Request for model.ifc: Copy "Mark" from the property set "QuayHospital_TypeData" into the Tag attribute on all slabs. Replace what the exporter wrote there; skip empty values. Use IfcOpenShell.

First a look at what the model holds.

```python
import ifcopenshell
import ifcopenshell.util.element

model = ifcopenshell.open("model.ifc")
print(model.schema)
slabs = model.by_type("IfcSlab")
print(len(slabs), "slabs")
for e in slabs[:8]:
    source = ifcopenshell.util.element.get_pset(e, "QuayHospital_TypeData", "Mark")
    target = e.Tag
    print(e.id(), repr(source), repr(target), sep=" | ")
```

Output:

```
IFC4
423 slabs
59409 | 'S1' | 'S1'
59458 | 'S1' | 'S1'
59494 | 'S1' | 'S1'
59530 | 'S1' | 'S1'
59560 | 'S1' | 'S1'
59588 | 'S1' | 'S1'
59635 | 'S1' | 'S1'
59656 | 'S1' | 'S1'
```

```python
import ifcopenshell
import ifcopenshell.util.element

model = ifcopenshell.open("model.ifc")

count = 0
for e in model.by_type("IfcSlab"):
    value = ifcopenshell.util.element.get_pset(e, "QuayHospital_TypeData", "Mark")
    current = e.Tag
    if not value or not value.strip() or current == value:
        continue
    e.Tag = value
    count += 1

print(count, "slabs updated")

model.write("model_updated.ifc")
```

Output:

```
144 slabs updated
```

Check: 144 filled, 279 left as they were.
